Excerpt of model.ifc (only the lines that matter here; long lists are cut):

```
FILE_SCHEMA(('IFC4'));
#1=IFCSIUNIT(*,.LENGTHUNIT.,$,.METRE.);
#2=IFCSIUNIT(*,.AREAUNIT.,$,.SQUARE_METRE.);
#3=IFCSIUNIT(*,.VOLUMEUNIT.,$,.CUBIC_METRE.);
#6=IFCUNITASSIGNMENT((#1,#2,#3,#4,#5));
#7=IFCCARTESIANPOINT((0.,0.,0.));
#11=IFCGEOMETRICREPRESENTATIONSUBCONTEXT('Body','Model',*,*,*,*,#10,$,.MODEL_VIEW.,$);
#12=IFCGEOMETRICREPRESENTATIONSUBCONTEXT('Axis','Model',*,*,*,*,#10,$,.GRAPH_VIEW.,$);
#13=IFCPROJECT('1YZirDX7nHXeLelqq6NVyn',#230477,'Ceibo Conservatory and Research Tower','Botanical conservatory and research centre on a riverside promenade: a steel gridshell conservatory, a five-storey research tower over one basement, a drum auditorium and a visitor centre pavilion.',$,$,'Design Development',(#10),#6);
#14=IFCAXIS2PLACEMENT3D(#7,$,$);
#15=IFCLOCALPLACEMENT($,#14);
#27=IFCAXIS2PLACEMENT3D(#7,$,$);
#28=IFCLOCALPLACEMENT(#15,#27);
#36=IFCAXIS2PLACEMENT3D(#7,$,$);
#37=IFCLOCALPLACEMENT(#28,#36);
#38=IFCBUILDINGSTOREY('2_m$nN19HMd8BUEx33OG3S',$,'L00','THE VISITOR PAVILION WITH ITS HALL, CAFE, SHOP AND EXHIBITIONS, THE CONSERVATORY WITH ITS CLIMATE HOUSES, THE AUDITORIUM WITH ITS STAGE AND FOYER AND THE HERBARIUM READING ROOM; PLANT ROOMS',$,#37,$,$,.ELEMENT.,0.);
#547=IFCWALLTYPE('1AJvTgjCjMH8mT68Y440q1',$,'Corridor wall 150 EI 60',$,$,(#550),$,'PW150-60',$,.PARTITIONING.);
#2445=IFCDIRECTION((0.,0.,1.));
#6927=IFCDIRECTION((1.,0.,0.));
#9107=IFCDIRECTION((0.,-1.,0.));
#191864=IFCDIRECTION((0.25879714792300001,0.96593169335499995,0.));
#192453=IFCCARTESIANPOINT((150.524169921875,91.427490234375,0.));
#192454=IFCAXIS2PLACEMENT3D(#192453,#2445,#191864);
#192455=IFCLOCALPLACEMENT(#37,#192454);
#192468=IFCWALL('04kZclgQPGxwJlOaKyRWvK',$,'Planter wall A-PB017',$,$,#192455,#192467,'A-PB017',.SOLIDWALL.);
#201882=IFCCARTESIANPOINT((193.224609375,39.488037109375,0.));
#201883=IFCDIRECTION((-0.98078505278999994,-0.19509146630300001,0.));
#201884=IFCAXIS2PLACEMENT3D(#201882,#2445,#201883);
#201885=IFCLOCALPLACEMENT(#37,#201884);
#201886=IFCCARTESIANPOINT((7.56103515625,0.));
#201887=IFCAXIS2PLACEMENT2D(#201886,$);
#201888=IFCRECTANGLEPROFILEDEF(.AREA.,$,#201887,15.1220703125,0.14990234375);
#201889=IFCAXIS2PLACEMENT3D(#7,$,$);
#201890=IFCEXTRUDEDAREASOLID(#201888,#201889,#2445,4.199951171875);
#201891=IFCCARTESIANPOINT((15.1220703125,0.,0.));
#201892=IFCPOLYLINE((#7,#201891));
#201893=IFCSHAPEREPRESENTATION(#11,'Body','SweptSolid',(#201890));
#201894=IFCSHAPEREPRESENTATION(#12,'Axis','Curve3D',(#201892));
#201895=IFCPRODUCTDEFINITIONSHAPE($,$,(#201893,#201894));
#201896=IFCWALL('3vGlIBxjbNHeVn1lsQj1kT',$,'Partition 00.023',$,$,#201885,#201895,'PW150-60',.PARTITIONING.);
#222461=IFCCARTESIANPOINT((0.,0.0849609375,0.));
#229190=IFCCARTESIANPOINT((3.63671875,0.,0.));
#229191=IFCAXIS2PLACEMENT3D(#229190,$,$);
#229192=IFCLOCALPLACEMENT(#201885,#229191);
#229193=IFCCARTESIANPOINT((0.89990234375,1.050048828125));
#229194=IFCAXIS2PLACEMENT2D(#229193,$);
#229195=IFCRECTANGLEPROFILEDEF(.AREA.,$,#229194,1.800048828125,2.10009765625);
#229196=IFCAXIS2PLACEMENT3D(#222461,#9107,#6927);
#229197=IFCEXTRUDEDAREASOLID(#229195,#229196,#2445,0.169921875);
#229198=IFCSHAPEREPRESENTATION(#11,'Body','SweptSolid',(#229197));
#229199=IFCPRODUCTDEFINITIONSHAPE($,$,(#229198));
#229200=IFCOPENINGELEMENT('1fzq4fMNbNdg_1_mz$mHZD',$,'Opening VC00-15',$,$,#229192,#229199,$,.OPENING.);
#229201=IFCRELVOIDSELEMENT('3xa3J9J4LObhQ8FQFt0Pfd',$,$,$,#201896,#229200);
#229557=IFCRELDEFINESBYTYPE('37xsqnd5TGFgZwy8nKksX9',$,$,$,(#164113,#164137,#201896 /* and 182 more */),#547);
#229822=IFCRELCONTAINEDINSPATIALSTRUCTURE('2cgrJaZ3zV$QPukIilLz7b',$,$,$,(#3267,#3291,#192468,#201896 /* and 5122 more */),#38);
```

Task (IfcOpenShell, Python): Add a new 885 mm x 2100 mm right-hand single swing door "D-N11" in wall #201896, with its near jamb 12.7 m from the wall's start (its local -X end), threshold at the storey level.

```python
import numpy as np
import ifcopenshell
import ifcopenshell.api.feature
import ifcopenshell.api.geometry
import ifcopenshell.api.root
import ifcopenshell.api.spatial
import ifcopenshell.geom
import ifcopenshell.util.element
import ifcopenshell.util.placement
import ifcopenshell.util.representation
import ifcopenshell.util.shape
import ifcopenshell.util.unit

model = ifcopenshell.open("model.ifc")
unit_scale = ifcopenshell.util.unit.calculate_unit_scale(model)
settings = ifcopenshell.geom.settings()


def volume(element):
    """Net volume in cubic metres, openings subtracted."""
    shape = ifcopenshell.geom.create_shape(settings, element)
    return ifcopenshell.util.shape.get_volume(shape.geometry)


wall = model.by_guid("3vGlIBxjbNHeVn1lsQj1kT")
storey = ifcopenshell.util.element.get_container(wall, ifc_class="IfcBuildingStorey")
context = ifcopenshell.util.representation.get_context(model, "Model", "Body", "MODEL_VIEW")
before = volume(wall)

width, height, from_end, sill = 0.885, 2.1, 12.7, 0.0  # metres

# The wall runs along its own X axis, and the end named is its -X end.
wall_shape = ifcopenshell.geom.create_shape(settings, wall)
x, y, z = ifcopenshell.util.shape.get_vertices(wall_shape.geometry).T
start = x.min() + from_end
face, thickness = float(y.min()), float(y.max() - y.min())
wall_matrix = ifcopenshell.util.placement.get_local_placement(wall.ObjectPlacement)
level = ifcopenshell.util.placement.get_local_placement(storey.ObjectPlacement)[2, 3]


def in_wall(x, y):
    """Placement at x, y metres in the wall's axes, at sill height."""
    matrix = wall_matrix.copy()
    matrix[:, 3] = wall_matrix @ np.array([x / unit_scale, y / unit_scale, 0.0, 1.0])
    matrix[2, 3] = level + sill / unit_scale
    return matrix


# Opening: a box that overshoots both wall faces by 50 mm.
opening = ifcopenshell.api.root.create_entity(model, ifc_class="IfcOpeningElement", predefined_type="OPENING")
box = ifcopenshell.api.geometry.add_wall_representation(
    model, context=context, length=width, height=height, thickness=thickness + 0.1
)
ifcopenshell.api.geometry.assign_representation(model, product=opening, representation=box)
ifcopenshell.api.geometry.edit_object_placement(model, product=opening, matrix=in_wall(start, face - 0.05), is_si=False)
ifcopenshell.api.feature.add_feature(model, feature=opening, element=wall)

door = ifcopenshell.api.root.create_entity(model, ifc_class="IfcDoor", name="D-N11", predefined_type="DOOR")
door.OverallWidth, door.OverallHeight = width / unit_scale, height / unit_scale
door.OperationType = "SINGLE_SWING_RIGHT"
body = ifcopenshell.api.geometry.add_door_representation(
    model,
    context=context,
    overall_width=door.OverallWidth,
    overall_height=door.OverallHeight,
    operation_type="SINGLE_SWING_RIGHT",
    lining_properties={"LiningDepth": thickness / unit_scale, "ThresholdDepth": thickness / unit_scale},
)
ifcopenshell.api.geometry.assign_representation(model, product=door, representation=body)
ifcopenshell.api.spatial.assign_container(model, products=[door], relating_structure=storey)
ifcopenshell.api.feature.add_filling(model, opening=opening, element=door)

# The lining spans the wall, so the door starts at the wall face.
ifcopenshell.api.geometry.edit_object_placement(model, product=door, matrix=in_wall(start, face), is_si=False)

after = volume(wall)

print(f"wall volume {before:.3f} -> {after:.3f} m3")

model.write("model_v2.ifc")
```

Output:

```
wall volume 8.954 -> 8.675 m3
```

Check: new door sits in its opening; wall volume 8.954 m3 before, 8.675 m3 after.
